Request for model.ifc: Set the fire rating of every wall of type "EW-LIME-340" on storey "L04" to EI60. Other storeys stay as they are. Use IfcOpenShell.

First a look at what the model holds.

```python
import ifcopenshell
import ifcopenshell.util.element

model = ifcopenshell.open("model.ifc")
print(model.schema)
storey = next(s for s in model.by_type("IfcBuildingStorey") if s.Name == "L04")
walls = [e for e in ifcopenshell.util.element.get_decomposition(storey) if e.is_a("IfcWall")]
seen = {}
for e in walls:
    element_type = ifcopenshell.util.element.get_type(e)
    key = (element_type.Name if element_type != e and element_type else None, ifcopenshell.util.element.get_pset(e, "Pset_WallCommon", "FireRating"))
    seen[key] = seen.get(key, 0) + 1
for (name, value), count in sorted(seen.items(), key=str):
    print(count, "x", name, "|", value)
```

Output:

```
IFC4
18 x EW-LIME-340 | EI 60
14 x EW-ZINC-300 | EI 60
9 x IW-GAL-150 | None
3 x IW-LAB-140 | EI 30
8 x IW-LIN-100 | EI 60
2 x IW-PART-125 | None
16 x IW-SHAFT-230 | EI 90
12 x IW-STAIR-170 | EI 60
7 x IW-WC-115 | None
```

```python
import ifcopenshell
import ifcopenshell.api.pset
import ifcopenshell.util.element

model = ifcopenshell.open("model.ifc")

storey = next(s for s in model.by_type("IfcBuildingStorey") if s.Name == "L04")
walls = [e for e in ifcopenshell.util.element.get_decomposition(storey) if e.is_a("IfcWall")]

count = 0
for e in walls:
    element_type = ifcopenshell.util.element.get_type(e)
    if element_type in (None, e) or element_type.Name != "EW-LIME-340":
        continue
    # add_pset returns the element's existing set when there is one.
    pset = ifcopenshell.api.pset.add_pset(model, product=e, name="Pset_WallCommon")
    ifcopenshell.api.pset.edit_pset(model, pset=pset, properties={"FireRating": "EI60"})
    count += 1

print(count, "walls updated")

model.write("model_v2.ifc")
```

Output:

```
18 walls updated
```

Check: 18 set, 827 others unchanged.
